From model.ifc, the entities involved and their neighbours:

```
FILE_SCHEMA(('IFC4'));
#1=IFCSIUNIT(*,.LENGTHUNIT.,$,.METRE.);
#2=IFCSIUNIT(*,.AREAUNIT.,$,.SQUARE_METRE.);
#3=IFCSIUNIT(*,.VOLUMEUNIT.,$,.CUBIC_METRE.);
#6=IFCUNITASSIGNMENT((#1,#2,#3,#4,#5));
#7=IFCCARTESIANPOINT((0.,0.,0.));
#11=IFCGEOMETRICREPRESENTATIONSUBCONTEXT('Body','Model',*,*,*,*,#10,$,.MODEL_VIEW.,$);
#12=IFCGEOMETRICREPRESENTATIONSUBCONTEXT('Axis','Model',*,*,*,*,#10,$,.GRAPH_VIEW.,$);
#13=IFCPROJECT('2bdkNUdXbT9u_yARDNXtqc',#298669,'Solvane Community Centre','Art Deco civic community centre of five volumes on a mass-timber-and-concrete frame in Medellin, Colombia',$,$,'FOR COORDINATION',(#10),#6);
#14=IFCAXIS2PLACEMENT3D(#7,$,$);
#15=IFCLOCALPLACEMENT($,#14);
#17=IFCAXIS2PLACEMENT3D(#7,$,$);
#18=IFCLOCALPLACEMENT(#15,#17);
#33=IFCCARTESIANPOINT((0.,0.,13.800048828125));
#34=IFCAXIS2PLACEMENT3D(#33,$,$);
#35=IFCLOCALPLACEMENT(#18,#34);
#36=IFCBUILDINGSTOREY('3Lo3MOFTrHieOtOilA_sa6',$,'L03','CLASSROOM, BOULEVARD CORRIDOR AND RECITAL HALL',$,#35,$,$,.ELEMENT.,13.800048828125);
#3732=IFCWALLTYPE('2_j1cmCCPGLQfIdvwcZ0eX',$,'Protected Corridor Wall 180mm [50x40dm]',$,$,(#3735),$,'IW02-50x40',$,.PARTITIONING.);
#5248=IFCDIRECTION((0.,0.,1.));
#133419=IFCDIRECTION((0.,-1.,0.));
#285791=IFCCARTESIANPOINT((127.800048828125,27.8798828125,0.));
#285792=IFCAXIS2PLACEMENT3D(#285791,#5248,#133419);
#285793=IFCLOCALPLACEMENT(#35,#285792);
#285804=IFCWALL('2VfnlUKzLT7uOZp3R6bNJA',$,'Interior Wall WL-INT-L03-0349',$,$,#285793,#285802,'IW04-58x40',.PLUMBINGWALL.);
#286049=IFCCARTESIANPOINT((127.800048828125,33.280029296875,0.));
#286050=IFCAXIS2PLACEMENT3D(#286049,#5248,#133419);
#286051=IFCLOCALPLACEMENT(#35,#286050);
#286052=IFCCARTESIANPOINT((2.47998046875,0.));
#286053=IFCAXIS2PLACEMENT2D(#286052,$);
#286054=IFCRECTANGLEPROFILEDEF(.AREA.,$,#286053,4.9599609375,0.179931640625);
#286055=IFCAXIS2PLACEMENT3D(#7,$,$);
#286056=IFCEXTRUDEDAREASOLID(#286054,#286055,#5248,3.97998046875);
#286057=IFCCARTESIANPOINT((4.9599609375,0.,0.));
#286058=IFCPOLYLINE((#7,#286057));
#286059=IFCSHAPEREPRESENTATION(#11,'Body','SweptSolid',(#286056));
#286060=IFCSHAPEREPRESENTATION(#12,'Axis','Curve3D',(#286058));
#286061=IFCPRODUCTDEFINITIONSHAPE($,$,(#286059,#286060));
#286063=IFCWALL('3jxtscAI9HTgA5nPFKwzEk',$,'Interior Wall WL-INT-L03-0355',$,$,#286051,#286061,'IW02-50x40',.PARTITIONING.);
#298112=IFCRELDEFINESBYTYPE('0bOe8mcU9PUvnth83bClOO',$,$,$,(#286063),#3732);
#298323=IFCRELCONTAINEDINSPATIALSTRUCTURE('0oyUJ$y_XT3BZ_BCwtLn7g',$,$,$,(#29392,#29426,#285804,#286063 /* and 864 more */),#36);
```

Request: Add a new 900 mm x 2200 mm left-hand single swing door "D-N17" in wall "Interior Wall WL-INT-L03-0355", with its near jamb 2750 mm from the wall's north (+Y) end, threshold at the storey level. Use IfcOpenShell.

```python
import numpy as np
import ifcopenshell
import ifcopenshell.api.feature
import ifcopenshell.api.geometry
import ifcopenshell.api.root
import ifcopenshell.api.spatial
import ifcopenshell.geom
import ifcopenshell.util.element
import ifcopenshell.util.placement
import ifcopenshell.util.representation
import ifcopenshell.util.shape
import ifcopenshell.util.unit

model = ifcopenshell.open("model.ifc")
unit_scale = ifcopenshell.util.unit.calculate_unit_scale(model)
settings = ifcopenshell.geom.settings()


def volume(element):
    """Net volume in cubic metres, openings subtracted."""
    shape = ifcopenshell.geom.create_shape(settings, element)
    return ifcopenshell.util.shape.get_volume(shape.geometry)


wall = model.by_guid("3jxtscAI9HTgA5nPFKwzEk")
storey = ifcopenshell.util.element.get_container(wall, ifc_class="IfcBuildingStorey")
context = ifcopenshell.util.representation.get_context(model, "Model", "Body", "MODEL_VIEW")
before = volume(wall)

width, height, from_end, sill = 0.9, 2.2, 2.75, 0.0  # metres

# The wall runs along its own X axis, and the end named is its -X end.
wall_shape = ifcopenshell.geom.create_shape(settings, wall)
x, y, z = ifcopenshell.util.shape.get_vertices(wall_shape.geometry).T
start = x.min() + from_end
face, thickness = float(y.min()), float(y.max() - y.min())
wall_matrix = ifcopenshell.util.placement.get_local_placement(wall.ObjectPlacement)
level = ifcopenshell.util.placement.get_local_placement(storey.ObjectPlacement)[2, 3]


def in_wall(x, y):
    """Placement at x, y metres in the wall's axes, at sill height."""
    matrix = wall_matrix.copy()
    matrix[:, 3] = wall_matrix @ np.array([x / unit_scale, y / unit_scale, 0.0, 1.0])
    matrix[2, 3] = level + sill / unit_scale
    return matrix


# Opening: a box that overshoots both wall faces by 50 mm.
opening = ifcopenshell.api.root.create_entity(model, ifc_class="IfcOpeningElement", predefined_type="OPENING")
box = ifcopenshell.api.geometry.add_wall_representation(
    model, context=context, length=width, height=height, thickness=thickness + 0.1
)
ifcopenshell.api.geometry.assign_representation(model, product=opening, representation=box)
ifcopenshell.api.geometry.edit_object_placement(model, product=opening, matrix=in_wall(start, face - 0.05), is_si=False)
ifcopenshell.api.feature.add_feature(model, feature=opening, element=wall)

door = ifcopenshell.api.root.create_entity(model, ifc_class="IfcDoor", name="D-N17", predefined_type="DOOR")
door.OverallWidth, door.OverallHeight = width / unit_scale, height / unit_scale
door.OperationType = "SINGLE_SWING_LEFT"
body = ifcopenshell.api.geometry.add_door_representation(
    model,
    context=context,
    overall_width=door.OverallWidth,
    overall_height=door.OverallHeight,
    operation_type="SINGLE_SWING_LEFT",
    lining_properties={"LiningDepth": thickness / unit_scale, "ThresholdDepth": thickness / unit_scale},
)
ifcopenshell.api.geometry.assign_representation(model, product=door, representation=body)
ifcopenshell.api.spatial.assign_container(model, products=[door], relating_structure=storey)
ifcopenshell.api.feature.add_filling(model, opening=opening, element=door)

# The lining spans the wall, so the door starts at the wall face.
ifcopenshell.api.geometry.edit_object_placement(model, product=door, matrix=in_wall(start, face), is_si=False)

after = volume(wall)

print(f"wall volume {before:.3f} -> {after:.3f} m3")

model.write("model_rev.ifc")
```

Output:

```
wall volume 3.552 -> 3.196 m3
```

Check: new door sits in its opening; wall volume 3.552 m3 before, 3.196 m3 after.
